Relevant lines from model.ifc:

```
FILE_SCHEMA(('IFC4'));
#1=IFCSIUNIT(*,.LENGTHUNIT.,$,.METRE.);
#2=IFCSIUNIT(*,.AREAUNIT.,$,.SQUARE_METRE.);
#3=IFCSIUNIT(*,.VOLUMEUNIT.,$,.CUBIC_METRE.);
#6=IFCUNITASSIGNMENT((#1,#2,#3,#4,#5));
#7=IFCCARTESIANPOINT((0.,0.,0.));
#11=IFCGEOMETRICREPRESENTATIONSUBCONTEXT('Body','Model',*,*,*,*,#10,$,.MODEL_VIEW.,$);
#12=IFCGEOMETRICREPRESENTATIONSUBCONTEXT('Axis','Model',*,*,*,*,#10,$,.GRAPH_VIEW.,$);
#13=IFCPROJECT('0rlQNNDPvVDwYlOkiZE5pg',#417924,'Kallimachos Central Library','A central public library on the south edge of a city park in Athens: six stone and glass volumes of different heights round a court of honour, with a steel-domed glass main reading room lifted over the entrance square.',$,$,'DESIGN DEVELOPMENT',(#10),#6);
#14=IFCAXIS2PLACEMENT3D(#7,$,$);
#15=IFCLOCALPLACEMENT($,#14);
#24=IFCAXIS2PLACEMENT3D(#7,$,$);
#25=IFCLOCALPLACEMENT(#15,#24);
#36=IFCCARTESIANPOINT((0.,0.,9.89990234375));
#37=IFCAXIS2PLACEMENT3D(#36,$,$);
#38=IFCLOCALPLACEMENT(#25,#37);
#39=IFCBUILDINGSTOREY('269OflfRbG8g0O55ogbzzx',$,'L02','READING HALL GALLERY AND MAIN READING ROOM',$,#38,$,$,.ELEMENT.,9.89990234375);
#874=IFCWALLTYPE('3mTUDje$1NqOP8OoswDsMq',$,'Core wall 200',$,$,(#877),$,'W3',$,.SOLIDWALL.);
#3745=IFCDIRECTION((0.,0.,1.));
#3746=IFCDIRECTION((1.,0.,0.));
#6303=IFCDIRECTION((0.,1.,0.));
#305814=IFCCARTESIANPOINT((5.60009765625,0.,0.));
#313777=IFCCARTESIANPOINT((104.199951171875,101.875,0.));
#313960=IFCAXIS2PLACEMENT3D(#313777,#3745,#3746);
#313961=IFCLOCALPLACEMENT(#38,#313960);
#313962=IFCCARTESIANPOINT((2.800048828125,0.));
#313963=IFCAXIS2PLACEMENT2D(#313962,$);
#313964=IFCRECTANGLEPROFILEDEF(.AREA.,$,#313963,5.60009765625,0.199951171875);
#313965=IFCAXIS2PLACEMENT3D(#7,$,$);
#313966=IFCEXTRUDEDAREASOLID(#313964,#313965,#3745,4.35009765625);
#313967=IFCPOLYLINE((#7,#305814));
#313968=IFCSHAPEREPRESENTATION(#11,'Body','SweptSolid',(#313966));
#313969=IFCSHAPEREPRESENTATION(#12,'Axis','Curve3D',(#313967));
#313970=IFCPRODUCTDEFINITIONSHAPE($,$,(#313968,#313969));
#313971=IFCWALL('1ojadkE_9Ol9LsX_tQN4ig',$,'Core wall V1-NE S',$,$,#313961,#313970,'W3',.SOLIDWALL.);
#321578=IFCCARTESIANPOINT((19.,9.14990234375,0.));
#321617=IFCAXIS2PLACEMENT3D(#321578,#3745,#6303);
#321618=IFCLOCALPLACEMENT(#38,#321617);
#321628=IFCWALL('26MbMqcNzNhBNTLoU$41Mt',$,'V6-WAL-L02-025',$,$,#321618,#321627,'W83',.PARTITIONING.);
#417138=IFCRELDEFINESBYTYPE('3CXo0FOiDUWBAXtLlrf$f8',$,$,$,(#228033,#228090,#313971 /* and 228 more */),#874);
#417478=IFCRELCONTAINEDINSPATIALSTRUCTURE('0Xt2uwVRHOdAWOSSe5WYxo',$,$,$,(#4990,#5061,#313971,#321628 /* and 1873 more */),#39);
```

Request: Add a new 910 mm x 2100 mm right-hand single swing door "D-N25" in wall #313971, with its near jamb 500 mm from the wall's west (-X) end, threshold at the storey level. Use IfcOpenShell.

```python
import numpy as np
import ifcopenshell
import ifcopenshell.api.feature
import ifcopenshell.api.geometry
import ifcopenshell.api.root
import ifcopenshell.api.spatial
import ifcopenshell.geom
import ifcopenshell.util.element
import ifcopenshell.util.placement
import ifcopenshell.util.representation
import ifcopenshell.util.shape
import ifcopenshell.util.unit

model = ifcopenshell.open("model.ifc")
unit_scale = ifcopenshell.util.unit.calculate_unit_scale(model)
settings = ifcopenshell.geom.settings()


def volume(element):
    """Net volume in cubic metres, openings subtracted."""
    shape = ifcopenshell.geom.create_shape(settings, element)
    return ifcopenshell.util.shape.get_volume(shape.geometry)


wall = model.by_guid("1ojadkE_9Ol9LsX_tQN4ig")
storey = ifcopenshell.util.element.get_container(wall, ifc_class="IfcBuildingStorey")
context = ifcopenshell.util.representation.get_context(model, "Model", "Body", "MODEL_VIEW")
before = volume(wall)

width, height, from_end, sill = 0.91, 2.1, 0.5, 0.0  # metres

# The wall runs along its own X axis, and the end named is its -X end.
wall_shape = ifcopenshell.geom.create_shape(settings, wall)
x, y, z = ifcopenshell.util.shape.get_vertices(wall_shape.geometry).T
start = x.min() + from_end
face, thickness = float(y.min()), float(y.max() - y.min())
wall_matrix = ifcopenshell.util.placement.get_local_placement(wall.ObjectPlacement)
level = ifcopenshell.util.placement.get_local_placement(storey.ObjectPlacement)[2, 3]


def in_wall(x, y):
    """Placement at x, y metres in the wall's axes, at sill height."""
    matrix = wall_matrix.copy()
    matrix[:, 3] = wall_matrix @ np.array([x / unit_scale, y / unit_scale, 0.0, 1.0])
    matrix[2, 3] = level + sill / unit_scale
    return matrix


# Opening: a box that overshoots both wall faces by 50 mm.
opening = ifcopenshell.api.root.create_entity(model, ifc_class="IfcOpeningElement", predefined_type="OPENING")
box = ifcopenshell.api.geometry.add_wall_representation(
    model, context=context, length=width, height=height, thickness=thickness + 0.1
)
ifcopenshell.api.geometry.assign_representation(model, product=opening, representation=box)
ifcopenshell.api.geometry.edit_object_placement(model, product=opening, matrix=in_wall(start, face - 0.05), is_si=False)
ifcopenshell.api.feature.add_feature(model, feature=opening, element=wall)

door = ifcopenshell.api.root.create_entity(model, ifc_class="IfcDoor", name="D-N25", predefined_type="DOOR")
door.OverallWidth, door.OverallHeight = width / unit_scale, height / unit_scale
door.OperationType = "SINGLE_SWING_RIGHT"
body = ifcopenshell.api.geometry.add_door_representation(
    model,
    context=context,
    overall_width=door.OverallWidth,
    overall_height=door.OverallHeight,
    operation_type="SINGLE_SWING_RIGHT",
    lining_properties={"LiningDepth": thickness / unit_scale, "ThresholdDepth": thickness / unit_scale},
)
ifcopenshell.api.geometry.assign_representation(model, product=door, representation=body)
ifcopenshell.api.spatial.assign_container(model, products=[door], relating_structure=storey)
ifcopenshell.api.feature.add_filling(model, opening=opening, element=door)

# The lining spans the wall, so the door starts at the wall face.
ifcopenshell.api.geometry.edit_object_placement(model, product=door, matrix=in_wall(start, face), is_si=False)

after = volume(wall)

print(f"wall volume {before:.3f} -> {after:.3f} m3")

model.write("model-out.ifc")
```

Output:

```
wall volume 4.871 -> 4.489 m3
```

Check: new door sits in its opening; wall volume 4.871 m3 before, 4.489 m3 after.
